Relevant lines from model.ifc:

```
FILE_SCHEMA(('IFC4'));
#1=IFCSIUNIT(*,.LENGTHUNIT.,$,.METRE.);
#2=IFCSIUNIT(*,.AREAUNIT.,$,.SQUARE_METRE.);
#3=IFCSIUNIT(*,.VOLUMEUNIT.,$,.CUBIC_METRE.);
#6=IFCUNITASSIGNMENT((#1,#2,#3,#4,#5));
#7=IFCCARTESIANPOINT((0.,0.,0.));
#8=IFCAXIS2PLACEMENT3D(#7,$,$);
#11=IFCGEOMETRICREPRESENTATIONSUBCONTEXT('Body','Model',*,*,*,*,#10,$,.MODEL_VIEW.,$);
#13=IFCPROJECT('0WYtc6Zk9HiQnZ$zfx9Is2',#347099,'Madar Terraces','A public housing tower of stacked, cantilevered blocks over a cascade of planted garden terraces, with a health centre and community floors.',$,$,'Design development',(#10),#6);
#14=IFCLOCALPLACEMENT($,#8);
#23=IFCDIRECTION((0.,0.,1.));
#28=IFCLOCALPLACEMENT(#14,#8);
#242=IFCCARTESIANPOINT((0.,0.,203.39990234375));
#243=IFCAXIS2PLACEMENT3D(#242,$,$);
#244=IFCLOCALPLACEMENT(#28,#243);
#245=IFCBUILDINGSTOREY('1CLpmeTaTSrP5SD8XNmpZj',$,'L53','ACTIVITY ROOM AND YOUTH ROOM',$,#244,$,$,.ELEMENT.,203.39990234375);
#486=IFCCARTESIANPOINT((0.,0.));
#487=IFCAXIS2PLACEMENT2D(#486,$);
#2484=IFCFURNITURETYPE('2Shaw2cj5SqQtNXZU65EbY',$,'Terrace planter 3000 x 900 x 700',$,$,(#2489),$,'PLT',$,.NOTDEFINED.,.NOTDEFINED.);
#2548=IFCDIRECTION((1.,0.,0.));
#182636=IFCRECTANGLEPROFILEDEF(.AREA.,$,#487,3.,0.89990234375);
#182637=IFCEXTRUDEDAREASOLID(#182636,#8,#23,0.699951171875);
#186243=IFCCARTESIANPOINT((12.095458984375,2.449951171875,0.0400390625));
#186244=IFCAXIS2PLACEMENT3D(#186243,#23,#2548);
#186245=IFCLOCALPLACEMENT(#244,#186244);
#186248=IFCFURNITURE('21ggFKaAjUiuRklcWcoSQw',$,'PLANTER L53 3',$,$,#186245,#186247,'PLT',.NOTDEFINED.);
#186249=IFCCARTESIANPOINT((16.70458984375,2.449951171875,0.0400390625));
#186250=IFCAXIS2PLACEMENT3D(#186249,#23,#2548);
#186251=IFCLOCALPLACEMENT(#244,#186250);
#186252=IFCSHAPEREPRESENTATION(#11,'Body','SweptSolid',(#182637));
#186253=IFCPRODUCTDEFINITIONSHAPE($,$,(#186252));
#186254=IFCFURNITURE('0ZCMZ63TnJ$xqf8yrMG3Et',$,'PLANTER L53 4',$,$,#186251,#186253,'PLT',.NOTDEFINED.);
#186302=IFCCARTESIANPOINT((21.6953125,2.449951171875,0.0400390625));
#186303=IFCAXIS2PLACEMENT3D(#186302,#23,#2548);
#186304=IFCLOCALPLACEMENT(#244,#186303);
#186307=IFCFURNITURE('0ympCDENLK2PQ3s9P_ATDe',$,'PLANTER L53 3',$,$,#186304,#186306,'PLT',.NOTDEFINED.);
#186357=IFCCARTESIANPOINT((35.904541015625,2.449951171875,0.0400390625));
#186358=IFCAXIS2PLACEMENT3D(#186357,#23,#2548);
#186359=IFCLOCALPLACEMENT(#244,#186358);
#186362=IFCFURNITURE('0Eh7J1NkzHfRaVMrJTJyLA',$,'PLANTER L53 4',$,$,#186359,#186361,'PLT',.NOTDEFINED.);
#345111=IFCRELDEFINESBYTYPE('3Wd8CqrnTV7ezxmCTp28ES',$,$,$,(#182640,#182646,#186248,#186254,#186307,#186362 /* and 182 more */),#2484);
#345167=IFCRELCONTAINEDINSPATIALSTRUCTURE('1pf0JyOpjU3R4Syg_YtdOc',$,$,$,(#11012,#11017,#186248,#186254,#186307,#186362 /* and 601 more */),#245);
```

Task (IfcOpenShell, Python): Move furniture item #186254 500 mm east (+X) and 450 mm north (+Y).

```python
import ifcopenshell
import ifcopenshell.api.geometry
import ifcopenshell.util.placement

model = ifcopenshell.open("model.ifc")

item = model.by_id(186254)
matrix = ifcopenshell.util.placement.get_local_placement(item.ObjectPlacement)
matrix[0, 3] += 0.5
matrix[1, 3] += 0.45
ifcopenshell.api.geometry.edit_object_placement(model, product=item, matrix=matrix, is_si=False)

print(ifcopenshell.util.placement.get_local_placement(item.ObjectPlacement).round(3) + 0.0)

model.write("model-out.ifc")
```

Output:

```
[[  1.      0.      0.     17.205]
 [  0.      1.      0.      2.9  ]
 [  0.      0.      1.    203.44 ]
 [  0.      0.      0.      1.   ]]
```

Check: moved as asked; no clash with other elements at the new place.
